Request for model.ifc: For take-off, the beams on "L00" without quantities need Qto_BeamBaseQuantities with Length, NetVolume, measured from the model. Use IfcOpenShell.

First a look at what the model holds.

```python
import ifcopenshell
import ifcopenshell.util.element
import ifcopenshell.util.unit

model = ifcopenshell.open("model.ifc")
print(model.schema)
for unit_type in ("LENGTHUNIT", "AREAUNIT", "VOLUMEUNIT"):
    print(unit_type, ifcopenshell.util.unit.calculate_unit_scale(model, unit_type))
storey = next(s for s in model.by_type("IfcBuildingStorey") if s.Name == "L00")
beams = [e for e in ifcopenshell.util.element.get_decomposition(storey) if e.is_a("IfcBeam")]
for e in sorted(beams, key=lambda e: e.id()):
    print(e.id(), e.is_a(), e.Name, list(ifcopenshell.util.element.get_psets(e, qtos_only=True)), sep=" | ")
```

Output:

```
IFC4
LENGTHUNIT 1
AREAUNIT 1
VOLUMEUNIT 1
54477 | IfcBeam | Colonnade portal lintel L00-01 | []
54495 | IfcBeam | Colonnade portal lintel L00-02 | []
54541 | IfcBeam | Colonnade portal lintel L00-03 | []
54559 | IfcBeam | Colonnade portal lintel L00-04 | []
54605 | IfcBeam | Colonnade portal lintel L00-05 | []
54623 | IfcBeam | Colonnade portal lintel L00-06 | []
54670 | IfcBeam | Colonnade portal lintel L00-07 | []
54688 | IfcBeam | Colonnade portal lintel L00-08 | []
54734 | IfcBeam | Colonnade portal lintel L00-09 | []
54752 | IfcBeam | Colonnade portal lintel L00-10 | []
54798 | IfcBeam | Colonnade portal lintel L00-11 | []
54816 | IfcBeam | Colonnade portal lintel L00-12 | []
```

```python
import ifcopenshell
import ifcopenshell.api.pset
import ifcopenshell.geom
import ifcopenshell.util.element
import ifcopenshell.util.shape
import ifcopenshell.util.unit

model = ifcopenshell.open("model.ifc")
unit_scale = ifcopenshell.util.unit.calculate_unit_scale(model)
volume_scale = ifcopenshell.util.unit.calculate_unit_scale(model, "VOLUMEUNIT")
settings = ifcopenshell.geom.settings()

storey = next(s for s in model.by_type("IfcBuildingStorey") if s.Name == "L00")
beams = [e for e in ifcopenshell.util.element.get_decomposition(storey) if e.is_a("IfcBeam")]

for e in sorted(beams, key=lambda e: e.id()):
    if ifcopenshell.util.element.get_psets(e, qtos_only=True, should_inherit=False):
        continue
    # Geometry comes back in metres, in the element's own axes.
    shape = ifcopenshell.geom.create_shape(settings, e)
    values = {
        "Length": ifcopenshell.util.shape.get_max_xyz(shape.geometry) / unit_scale,
        "NetVolume": ifcopenshell.util.shape.get_volume(shape.geometry) / volume_scale,
    }
    qto = ifcopenshell.api.pset.add_qto(model, product=e, name="Qto_BeamBaseQuantities")
    ifcopenshell.api.pset.edit_qto(model, qto=qto, properties=values)
    print(e.id(), {k: round(v, 3) for k, v in values.items()})

model.write("model_rev.ifc")
```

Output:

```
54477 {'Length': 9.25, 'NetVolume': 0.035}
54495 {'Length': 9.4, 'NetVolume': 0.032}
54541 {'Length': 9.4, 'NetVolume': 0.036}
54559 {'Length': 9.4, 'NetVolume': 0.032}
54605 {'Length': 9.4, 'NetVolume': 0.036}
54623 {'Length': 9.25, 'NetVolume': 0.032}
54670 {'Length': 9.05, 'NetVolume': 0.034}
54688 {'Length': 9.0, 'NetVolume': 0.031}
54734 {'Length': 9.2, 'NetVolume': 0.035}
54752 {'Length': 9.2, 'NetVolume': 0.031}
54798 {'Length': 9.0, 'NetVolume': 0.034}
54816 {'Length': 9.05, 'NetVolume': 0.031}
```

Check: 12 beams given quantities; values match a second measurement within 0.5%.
